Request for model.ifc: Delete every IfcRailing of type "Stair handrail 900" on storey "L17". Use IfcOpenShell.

First a look at what the model holds.

```python
import ifcopenshell
import ifcopenshell.util.element

model = ifcopenshell.open("model.ifc")
print(model.schema)
storey = next(s for s in model.by_type("IfcBuildingStorey") if s.Name == "L17")
railings = [e for e in ifcopenshell.util.element.get_decomposition(storey) if e.is_a("IfcRailing")]
seen = {}
for e in railings:
    element_type = ifcopenshell.util.element.get_type(e)
    name = element_type.Name if element_type not in (None, e) else None
    seen[name] = seen.get(name, 0) + 1
for name, count in sorted(seen.items(), key=str):
    print(count, "x", name)
```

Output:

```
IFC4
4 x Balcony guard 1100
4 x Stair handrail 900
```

```python
import ifcopenshell
import ifcopenshell.api.root
import ifcopenshell.util.element

model = ifcopenshell.open("model.ifc")

storey = next(s for s in model.by_type("IfcBuildingStorey") if s.Name == "L17")
railings = [e for e in ifcopenshell.util.element.get_decomposition(storey) if e.is_a("IfcRailing")]
targets = [e for e in railings if (t := ifcopenshell.util.element.get_type(e)) not in (None, e) and t.Name == "Stair handrail 900"]

for e in targets:
    ifcopenshell.api.root.remove_product(model, product=e)
print(len(targets), "removed")

model.write("model-out.ifc")
```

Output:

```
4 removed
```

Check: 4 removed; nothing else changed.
